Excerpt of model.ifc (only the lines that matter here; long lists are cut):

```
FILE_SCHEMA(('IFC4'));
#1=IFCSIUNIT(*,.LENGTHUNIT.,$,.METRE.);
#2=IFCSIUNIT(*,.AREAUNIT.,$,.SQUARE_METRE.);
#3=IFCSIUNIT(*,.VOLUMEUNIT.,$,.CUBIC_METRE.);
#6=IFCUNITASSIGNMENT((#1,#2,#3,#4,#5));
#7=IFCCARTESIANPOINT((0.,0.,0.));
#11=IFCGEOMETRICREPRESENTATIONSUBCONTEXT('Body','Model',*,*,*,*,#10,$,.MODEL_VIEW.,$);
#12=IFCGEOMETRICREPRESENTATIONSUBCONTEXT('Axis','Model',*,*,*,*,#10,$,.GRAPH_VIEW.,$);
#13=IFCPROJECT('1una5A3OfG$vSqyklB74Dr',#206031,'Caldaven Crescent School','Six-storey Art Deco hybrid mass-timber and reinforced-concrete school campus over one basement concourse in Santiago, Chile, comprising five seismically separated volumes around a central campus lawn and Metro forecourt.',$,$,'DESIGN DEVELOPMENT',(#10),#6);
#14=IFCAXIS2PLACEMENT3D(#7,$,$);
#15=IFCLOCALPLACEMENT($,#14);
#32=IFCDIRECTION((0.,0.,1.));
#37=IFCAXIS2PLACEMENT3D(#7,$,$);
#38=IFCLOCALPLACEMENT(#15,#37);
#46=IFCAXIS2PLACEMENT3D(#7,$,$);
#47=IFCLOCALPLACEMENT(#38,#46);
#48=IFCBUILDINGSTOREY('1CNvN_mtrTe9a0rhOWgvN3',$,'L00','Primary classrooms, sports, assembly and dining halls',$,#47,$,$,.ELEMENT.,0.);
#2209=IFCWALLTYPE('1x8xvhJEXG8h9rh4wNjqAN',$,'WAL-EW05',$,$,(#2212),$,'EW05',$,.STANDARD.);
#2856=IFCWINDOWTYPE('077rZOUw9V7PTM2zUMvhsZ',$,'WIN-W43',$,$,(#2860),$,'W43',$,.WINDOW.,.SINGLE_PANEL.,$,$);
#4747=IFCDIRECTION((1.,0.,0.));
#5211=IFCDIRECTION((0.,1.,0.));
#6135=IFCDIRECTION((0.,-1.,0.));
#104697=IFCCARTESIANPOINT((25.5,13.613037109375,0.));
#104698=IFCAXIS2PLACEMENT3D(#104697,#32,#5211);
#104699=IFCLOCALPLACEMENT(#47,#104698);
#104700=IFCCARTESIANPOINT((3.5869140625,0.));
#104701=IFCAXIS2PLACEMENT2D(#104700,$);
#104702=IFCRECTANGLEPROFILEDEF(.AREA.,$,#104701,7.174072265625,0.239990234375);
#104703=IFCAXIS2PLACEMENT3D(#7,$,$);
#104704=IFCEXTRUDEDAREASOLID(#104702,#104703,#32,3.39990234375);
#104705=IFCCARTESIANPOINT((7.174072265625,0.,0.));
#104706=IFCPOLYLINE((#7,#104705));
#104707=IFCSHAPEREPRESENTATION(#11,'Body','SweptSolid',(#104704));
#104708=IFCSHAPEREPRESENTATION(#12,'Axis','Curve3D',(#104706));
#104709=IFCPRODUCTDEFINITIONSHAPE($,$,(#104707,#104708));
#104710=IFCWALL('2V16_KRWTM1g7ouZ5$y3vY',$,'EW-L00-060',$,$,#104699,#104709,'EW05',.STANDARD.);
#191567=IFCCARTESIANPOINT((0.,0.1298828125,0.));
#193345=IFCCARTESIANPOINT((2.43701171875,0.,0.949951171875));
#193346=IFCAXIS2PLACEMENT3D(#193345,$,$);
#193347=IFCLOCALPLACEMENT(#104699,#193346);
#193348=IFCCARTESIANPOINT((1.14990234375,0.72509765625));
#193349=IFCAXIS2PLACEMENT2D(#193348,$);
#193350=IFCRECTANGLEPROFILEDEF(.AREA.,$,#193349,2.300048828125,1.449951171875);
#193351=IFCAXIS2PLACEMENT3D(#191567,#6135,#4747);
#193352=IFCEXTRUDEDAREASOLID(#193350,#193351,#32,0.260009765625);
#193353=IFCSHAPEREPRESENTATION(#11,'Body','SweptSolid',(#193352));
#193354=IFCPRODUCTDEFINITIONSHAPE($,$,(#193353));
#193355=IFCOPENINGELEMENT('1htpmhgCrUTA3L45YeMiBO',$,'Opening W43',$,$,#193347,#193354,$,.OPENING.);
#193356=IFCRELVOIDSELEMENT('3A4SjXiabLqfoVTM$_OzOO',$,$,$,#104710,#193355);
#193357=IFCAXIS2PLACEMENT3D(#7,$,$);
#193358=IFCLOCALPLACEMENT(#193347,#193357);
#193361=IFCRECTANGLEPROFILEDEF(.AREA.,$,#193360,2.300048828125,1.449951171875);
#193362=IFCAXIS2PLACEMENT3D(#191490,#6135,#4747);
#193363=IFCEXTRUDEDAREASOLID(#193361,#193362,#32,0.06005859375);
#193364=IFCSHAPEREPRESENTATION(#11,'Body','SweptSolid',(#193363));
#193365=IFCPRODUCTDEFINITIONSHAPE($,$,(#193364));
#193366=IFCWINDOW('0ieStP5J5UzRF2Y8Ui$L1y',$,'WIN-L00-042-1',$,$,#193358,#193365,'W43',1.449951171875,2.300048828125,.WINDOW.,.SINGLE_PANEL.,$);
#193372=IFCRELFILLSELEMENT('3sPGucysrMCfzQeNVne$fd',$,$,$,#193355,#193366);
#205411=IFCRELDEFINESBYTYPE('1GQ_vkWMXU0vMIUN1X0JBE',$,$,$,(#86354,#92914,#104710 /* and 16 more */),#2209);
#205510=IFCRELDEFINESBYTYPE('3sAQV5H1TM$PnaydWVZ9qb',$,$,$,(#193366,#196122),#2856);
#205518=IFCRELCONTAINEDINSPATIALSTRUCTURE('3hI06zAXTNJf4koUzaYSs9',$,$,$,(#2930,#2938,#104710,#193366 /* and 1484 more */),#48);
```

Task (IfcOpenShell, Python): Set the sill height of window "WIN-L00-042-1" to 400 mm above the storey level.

```python
import numpy as np
import ifcopenshell
import ifcopenshell.api.geometry
import ifcopenshell.geom
import ifcopenshell.util.element
import ifcopenshell.util.placement
import ifcopenshell.util.shape
import ifcopenshell.util.unit

model = ifcopenshell.open("model.ifc")
unit_scale = ifcopenshell.util.unit.calculate_unit_scale(model)

window = model.by_id(193366)
opening = window.FillsVoids[0].RelatingOpeningElement
storey = ifcopenshell.util.element.get_container(window, ifc_class="IfcBuildingStorey")
level = ifcopenshell.util.placement.get_local_placement(storey.ObjectPlacement)[2, 3]

# The opening's origin need not be at the sill, so measure its lowest point.
shape = ifcopenshell.geom.create_shape(ifcopenshell.geom.settings(), opening)
bottom = ifcopenshell.util.shape.get_shape_bottom_elevation(shape, shape.geometry) / unit_scale
dz = level + 0.4 / unit_scale - bottom

shift = np.array([0.0, 0.0, dz])
# The window is placed relative to its opening, so it follows when the opening moves.
matrix = ifcopenshell.util.placement.get_local_placement(opening.ObjectPlacement)
matrix[:3, 3] += shift
ifcopenshell.api.geometry.edit_object_placement(
    model, product=opening, matrix=matrix, is_si=False, should_transform_children=True
)

print(f"moved by {dz * unit_scale:+.3f} m")

model.write("model_rev.ifc")
```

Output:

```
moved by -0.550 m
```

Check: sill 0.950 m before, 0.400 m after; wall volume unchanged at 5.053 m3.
